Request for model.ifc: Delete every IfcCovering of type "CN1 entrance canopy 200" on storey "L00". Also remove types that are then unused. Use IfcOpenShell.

First a look at what the model holds.

```python
import ifcopenshell
import ifcopenshell.util.element

model = ifcopenshell.open("model.ifc")
print(model.schema)
storey = next(s for s in model.by_type("IfcBuildingStorey") if s.Name == "L00")
coverings = [e for e in ifcopenshell.util.element.get_decomposition(storey) if e.is_a("IfcCovering")]
seen = {}
for e in coverings:
    element_type = ifcopenshell.util.element.get_type(e)
    name = element_type.Name if element_type not in (None, e) else None
    seen[name] = seen.get(name, 0) + 1
for name, count in sorted(seen.items(), key=str):
    print(count, "x", name)
```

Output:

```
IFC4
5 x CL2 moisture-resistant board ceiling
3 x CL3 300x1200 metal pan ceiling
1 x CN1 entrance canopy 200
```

```python
import ifcopenshell
import ifcopenshell.api.root
import ifcopenshell.util.element

model = ifcopenshell.open("model.ifc")

storey = next(s for s in model.by_type("IfcBuildingStorey") if s.Name == "L00")
coverings = [e for e in ifcopenshell.util.element.get_decomposition(storey) if e.is_a("IfcCovering")]
targets = [e for e in coverings if (t := ifcopenshell.util.element.get_type(e)) not in (None, e) and t.Name == "CN1 entrance canopy 200"]
types = {ifcopenshell.util.element.get_type(e) for e in targets} - {None, *targets}

for e in targets:
    ifcopenshell.api.root.remove_product(model, product=e)
print(len(targets), "removed")

unused = [t for t in types if not ifcopenshell.util.element.get_types(t)]
for t in unused:
    ifcopenshell.api.root.remove_product(model, product=t)
print(len(unused), "unused types removed")

model.write("model-out.ifc")
```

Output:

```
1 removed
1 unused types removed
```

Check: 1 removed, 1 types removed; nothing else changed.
